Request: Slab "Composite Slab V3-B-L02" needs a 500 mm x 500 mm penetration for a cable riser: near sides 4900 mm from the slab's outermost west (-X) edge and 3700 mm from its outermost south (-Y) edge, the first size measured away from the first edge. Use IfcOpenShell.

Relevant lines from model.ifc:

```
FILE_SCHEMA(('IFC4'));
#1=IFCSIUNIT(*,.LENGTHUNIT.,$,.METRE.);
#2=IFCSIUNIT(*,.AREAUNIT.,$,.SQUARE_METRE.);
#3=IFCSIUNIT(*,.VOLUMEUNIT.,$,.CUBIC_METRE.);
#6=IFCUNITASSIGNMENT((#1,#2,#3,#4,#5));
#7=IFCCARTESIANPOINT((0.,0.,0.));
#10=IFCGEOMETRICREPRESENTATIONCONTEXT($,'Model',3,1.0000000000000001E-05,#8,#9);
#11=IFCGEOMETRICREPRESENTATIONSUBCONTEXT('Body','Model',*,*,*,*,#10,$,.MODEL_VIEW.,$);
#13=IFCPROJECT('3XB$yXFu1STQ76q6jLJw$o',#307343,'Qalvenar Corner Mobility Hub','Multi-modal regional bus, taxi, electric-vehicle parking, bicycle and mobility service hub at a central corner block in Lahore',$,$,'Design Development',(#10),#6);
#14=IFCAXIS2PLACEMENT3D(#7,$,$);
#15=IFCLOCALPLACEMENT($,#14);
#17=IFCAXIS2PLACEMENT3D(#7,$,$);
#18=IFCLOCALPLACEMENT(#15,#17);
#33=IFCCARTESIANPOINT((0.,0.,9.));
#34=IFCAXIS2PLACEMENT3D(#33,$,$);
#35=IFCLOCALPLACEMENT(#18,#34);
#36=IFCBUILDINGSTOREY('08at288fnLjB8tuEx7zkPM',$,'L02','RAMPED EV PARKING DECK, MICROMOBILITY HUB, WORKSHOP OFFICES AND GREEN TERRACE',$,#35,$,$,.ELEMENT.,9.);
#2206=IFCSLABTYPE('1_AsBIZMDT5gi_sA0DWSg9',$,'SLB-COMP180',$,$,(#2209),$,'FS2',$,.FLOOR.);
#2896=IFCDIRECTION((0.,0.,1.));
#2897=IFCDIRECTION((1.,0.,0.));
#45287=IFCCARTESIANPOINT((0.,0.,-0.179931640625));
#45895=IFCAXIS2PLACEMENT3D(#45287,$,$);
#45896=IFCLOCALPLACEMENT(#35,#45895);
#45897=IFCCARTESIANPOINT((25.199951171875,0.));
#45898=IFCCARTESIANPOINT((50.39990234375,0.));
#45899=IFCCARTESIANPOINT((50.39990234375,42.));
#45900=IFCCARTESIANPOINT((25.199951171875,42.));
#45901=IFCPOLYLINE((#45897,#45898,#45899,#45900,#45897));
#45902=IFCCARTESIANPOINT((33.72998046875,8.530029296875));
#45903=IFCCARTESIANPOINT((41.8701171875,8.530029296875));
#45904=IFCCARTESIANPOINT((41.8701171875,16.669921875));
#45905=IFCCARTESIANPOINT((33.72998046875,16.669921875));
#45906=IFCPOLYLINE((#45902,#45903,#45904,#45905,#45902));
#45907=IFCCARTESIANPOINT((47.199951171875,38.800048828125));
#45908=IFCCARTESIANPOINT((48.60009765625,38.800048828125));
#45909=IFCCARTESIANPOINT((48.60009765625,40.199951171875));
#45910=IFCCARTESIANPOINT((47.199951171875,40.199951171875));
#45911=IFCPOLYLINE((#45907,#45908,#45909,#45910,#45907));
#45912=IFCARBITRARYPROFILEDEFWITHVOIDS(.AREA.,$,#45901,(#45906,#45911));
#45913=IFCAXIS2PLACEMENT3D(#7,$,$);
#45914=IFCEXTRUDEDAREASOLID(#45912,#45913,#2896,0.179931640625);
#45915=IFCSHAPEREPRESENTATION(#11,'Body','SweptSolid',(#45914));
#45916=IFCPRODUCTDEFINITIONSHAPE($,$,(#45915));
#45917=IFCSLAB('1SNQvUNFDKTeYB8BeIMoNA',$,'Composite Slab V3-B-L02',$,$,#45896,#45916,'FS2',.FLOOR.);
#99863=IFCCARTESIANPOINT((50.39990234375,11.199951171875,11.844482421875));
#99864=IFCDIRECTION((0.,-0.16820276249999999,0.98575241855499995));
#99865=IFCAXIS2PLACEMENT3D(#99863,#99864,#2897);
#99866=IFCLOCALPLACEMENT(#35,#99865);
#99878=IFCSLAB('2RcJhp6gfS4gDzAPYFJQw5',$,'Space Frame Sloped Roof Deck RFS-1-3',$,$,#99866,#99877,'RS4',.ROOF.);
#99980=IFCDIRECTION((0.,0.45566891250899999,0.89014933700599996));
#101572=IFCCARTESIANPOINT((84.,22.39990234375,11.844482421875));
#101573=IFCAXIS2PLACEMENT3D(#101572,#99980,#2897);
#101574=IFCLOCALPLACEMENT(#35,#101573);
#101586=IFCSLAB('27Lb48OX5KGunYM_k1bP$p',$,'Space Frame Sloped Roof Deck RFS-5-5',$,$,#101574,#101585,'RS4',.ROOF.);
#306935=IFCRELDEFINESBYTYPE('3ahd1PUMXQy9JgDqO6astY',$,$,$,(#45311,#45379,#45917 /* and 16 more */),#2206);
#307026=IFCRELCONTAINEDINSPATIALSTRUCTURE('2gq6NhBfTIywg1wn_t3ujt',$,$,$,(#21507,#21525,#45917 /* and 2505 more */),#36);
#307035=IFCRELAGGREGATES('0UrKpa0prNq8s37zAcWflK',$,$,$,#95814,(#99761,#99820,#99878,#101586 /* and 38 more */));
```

```python
import numpy as np
import ifcopenshell
import ifcopenshell.api.feature
import ifcopenshell.api.geometry
import ifcopenshell.api.root
import ifcopenshell.geom
import ifcopenshell.util.placement
import ifcopenshell.util.representation
import ifcopenshell.util.shape
import ifcopenshell.util.unit

model = ifcopenshell.open("model.ifc")
unit_scale = ifcopenshell.util.unit.calculate_unit_scale(model)
settings = ifcopenshell.geom.settings()


def volume(element):
    """Net volume in cubic metres, openings subtracted."""
    shape = ifcopenshell.geom.create_shape(settings, element)
    return ifcopenshell.util.shape.get_volume(shape.geometry)


slab = model.by_guid("1SNQvUNFDKTeYB8BeIMoNA")
before = volume(slab)

# Extent in the slab's own axes, in metres. The edges named are its -X and -Y sides.
slab_shape = ifcopenshell.geom.create_shape(settings, slab)
vertices = ifcopenshell.util.shape.get_vertices(slab_shape.geometry)
x_min, y_min, bottom = vertices.min(axis=0)
top = vertices[:, 2].max()

opening = ifcopenshell.api.root.create_entity(model, ifc_class="IfcOpeningElement", name="Cable riser opening", predefined_type="OPENING")
context = ifcopenshell.util.representation.get_context(model, "Model", "Body", "MODEL_VIEW")
width, depth = 0.5, 0.5
outline = [(0.0, 0.0), (width, 0.0), (width, depth), (0.0, depth), (0.0, 0.0)]
# Overshoot both faces by 50 mm so the cut is clean.
shape = ifcopenshell.api.geometry.add_slab_representation(
    model, context=context, depth=top - bottom + 0.1, polyline=outline
)
ifcopenshell.api.geometry.assign_representation(model, product=opening, representation=shape)

matrix = ifcopenshell.util.placement.get_local_placement(slab.ObjectPlacement)
matrix[:, 3] = matrix @ np.append(np.array([x_min + 4.9, y_min + 3.7, bottom - 0.05]) / unit_scale, 1.0)
ifcopenshell.api.geometry.edit_object_placement(model, product=opening, matrix=matrix, is_si=False)
ifcopenshell.api.feature.add_feature(model, feature=opening, element=slab)

after = volume(slab)

print(f"slab volume {before:.3f} -> {after:.3f} m3")

model.write("model-out.ifc")
```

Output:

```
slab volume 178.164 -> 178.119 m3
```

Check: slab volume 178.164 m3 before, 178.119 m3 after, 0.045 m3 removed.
